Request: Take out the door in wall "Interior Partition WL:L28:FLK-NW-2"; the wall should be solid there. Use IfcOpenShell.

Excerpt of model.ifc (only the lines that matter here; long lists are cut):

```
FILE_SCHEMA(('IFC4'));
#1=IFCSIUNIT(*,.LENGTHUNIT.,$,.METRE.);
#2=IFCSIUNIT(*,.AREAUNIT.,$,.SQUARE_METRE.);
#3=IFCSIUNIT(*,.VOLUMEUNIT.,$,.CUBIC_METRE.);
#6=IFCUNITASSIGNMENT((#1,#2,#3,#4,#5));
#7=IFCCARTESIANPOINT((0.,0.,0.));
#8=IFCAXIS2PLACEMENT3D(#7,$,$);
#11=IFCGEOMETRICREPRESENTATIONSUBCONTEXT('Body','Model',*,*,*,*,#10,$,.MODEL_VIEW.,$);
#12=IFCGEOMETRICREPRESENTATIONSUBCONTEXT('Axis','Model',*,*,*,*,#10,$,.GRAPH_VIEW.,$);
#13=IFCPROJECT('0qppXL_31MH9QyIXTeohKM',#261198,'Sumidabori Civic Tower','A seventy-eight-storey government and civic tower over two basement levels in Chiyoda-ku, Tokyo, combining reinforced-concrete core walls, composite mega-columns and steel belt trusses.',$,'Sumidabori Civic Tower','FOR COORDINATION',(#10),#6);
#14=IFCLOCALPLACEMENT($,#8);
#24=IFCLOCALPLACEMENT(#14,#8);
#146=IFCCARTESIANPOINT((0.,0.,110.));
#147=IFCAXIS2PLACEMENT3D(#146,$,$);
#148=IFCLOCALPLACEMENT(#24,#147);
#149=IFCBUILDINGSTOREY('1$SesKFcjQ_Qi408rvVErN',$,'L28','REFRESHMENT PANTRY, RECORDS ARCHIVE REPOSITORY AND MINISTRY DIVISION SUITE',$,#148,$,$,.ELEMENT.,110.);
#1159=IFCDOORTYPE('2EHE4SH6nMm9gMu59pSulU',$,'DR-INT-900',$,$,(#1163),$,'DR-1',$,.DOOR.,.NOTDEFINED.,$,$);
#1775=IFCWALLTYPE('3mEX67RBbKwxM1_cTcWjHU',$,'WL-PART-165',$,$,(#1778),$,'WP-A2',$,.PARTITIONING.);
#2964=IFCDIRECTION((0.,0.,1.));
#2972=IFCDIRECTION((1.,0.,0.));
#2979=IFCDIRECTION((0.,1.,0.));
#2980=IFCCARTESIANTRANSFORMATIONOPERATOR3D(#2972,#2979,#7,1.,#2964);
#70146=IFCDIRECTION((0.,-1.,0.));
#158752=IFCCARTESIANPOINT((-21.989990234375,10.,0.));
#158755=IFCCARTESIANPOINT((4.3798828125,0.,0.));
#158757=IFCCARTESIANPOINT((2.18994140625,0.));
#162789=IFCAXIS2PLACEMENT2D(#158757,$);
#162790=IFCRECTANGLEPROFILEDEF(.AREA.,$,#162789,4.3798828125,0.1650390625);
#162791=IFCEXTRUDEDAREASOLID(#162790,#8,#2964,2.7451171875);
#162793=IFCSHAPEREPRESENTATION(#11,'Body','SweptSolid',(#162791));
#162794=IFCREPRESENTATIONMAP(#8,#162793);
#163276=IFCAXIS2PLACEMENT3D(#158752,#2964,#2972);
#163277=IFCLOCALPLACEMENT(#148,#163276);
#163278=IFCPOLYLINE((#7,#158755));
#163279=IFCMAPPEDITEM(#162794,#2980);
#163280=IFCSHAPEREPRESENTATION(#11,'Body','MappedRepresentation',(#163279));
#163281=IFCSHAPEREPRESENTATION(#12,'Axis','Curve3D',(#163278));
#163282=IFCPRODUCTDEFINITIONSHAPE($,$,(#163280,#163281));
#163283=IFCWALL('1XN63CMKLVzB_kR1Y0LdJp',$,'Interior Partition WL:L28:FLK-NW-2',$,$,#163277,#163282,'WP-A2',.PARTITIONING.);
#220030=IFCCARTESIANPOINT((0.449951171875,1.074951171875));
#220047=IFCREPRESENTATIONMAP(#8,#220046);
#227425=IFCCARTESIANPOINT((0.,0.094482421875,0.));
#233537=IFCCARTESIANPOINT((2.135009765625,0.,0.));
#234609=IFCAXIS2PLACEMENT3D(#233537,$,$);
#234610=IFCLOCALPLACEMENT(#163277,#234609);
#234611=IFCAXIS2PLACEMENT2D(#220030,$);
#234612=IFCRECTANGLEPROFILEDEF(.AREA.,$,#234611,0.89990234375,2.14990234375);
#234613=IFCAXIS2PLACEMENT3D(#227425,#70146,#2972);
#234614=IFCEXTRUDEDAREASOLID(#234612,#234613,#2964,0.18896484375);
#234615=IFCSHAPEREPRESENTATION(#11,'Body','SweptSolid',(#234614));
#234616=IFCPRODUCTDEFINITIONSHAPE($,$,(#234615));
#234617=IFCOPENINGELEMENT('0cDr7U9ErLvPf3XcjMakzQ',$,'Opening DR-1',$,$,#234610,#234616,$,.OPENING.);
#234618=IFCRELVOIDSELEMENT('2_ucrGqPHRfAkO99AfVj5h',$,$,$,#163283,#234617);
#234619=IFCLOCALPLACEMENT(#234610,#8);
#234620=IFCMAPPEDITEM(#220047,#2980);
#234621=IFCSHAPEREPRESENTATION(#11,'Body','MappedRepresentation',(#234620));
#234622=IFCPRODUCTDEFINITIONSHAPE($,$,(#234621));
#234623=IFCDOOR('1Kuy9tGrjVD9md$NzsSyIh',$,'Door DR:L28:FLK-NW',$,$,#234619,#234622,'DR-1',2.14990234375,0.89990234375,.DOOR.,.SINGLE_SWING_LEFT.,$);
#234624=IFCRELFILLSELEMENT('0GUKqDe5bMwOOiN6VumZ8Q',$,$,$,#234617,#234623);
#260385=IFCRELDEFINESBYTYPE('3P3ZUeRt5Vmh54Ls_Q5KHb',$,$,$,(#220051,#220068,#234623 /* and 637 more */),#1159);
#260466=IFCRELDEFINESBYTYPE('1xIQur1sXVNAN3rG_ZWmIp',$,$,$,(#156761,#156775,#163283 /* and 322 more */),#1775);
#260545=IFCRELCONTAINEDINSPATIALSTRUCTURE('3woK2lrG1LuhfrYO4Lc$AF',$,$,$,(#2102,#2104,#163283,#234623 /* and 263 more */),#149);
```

```python
import ifcopenshell
import ifcopenshell.api.feature
import ifcopenshell.api.root
import ifcopenshell.geom
import ifcopenshell.util.shape

model = ifcopenshell.open("model.ifc")
settings = ifcopenshell.geom.settings()


def volume(element):
    """Net volume in cubic metres, openings subtracted."""
    shape = ifcopenshell.geom.create_shape(settings, element)
    return ifcopenshell.util.shape.get_volume(shape.geometry)


door = model.by_guid("1Kuy9tGrjVD9md$NzsSyIh")
opening = door.FillsVoids[0].RelatingOpeningElement
wall = opening.VoidsElements[0].RelatingBuildingElement
before = volume(wall)

ifcopenshell.api.root.remove_product(model, product=door)
ifcopenshell.api.feature.remove_feature(model, feature=opening)

after = volume(wall)

print(f"wall volume {before:.3f} -> {after:.3f} m3")

model.write("model_edited.ifc")
```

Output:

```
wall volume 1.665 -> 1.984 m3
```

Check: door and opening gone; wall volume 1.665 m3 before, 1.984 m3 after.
